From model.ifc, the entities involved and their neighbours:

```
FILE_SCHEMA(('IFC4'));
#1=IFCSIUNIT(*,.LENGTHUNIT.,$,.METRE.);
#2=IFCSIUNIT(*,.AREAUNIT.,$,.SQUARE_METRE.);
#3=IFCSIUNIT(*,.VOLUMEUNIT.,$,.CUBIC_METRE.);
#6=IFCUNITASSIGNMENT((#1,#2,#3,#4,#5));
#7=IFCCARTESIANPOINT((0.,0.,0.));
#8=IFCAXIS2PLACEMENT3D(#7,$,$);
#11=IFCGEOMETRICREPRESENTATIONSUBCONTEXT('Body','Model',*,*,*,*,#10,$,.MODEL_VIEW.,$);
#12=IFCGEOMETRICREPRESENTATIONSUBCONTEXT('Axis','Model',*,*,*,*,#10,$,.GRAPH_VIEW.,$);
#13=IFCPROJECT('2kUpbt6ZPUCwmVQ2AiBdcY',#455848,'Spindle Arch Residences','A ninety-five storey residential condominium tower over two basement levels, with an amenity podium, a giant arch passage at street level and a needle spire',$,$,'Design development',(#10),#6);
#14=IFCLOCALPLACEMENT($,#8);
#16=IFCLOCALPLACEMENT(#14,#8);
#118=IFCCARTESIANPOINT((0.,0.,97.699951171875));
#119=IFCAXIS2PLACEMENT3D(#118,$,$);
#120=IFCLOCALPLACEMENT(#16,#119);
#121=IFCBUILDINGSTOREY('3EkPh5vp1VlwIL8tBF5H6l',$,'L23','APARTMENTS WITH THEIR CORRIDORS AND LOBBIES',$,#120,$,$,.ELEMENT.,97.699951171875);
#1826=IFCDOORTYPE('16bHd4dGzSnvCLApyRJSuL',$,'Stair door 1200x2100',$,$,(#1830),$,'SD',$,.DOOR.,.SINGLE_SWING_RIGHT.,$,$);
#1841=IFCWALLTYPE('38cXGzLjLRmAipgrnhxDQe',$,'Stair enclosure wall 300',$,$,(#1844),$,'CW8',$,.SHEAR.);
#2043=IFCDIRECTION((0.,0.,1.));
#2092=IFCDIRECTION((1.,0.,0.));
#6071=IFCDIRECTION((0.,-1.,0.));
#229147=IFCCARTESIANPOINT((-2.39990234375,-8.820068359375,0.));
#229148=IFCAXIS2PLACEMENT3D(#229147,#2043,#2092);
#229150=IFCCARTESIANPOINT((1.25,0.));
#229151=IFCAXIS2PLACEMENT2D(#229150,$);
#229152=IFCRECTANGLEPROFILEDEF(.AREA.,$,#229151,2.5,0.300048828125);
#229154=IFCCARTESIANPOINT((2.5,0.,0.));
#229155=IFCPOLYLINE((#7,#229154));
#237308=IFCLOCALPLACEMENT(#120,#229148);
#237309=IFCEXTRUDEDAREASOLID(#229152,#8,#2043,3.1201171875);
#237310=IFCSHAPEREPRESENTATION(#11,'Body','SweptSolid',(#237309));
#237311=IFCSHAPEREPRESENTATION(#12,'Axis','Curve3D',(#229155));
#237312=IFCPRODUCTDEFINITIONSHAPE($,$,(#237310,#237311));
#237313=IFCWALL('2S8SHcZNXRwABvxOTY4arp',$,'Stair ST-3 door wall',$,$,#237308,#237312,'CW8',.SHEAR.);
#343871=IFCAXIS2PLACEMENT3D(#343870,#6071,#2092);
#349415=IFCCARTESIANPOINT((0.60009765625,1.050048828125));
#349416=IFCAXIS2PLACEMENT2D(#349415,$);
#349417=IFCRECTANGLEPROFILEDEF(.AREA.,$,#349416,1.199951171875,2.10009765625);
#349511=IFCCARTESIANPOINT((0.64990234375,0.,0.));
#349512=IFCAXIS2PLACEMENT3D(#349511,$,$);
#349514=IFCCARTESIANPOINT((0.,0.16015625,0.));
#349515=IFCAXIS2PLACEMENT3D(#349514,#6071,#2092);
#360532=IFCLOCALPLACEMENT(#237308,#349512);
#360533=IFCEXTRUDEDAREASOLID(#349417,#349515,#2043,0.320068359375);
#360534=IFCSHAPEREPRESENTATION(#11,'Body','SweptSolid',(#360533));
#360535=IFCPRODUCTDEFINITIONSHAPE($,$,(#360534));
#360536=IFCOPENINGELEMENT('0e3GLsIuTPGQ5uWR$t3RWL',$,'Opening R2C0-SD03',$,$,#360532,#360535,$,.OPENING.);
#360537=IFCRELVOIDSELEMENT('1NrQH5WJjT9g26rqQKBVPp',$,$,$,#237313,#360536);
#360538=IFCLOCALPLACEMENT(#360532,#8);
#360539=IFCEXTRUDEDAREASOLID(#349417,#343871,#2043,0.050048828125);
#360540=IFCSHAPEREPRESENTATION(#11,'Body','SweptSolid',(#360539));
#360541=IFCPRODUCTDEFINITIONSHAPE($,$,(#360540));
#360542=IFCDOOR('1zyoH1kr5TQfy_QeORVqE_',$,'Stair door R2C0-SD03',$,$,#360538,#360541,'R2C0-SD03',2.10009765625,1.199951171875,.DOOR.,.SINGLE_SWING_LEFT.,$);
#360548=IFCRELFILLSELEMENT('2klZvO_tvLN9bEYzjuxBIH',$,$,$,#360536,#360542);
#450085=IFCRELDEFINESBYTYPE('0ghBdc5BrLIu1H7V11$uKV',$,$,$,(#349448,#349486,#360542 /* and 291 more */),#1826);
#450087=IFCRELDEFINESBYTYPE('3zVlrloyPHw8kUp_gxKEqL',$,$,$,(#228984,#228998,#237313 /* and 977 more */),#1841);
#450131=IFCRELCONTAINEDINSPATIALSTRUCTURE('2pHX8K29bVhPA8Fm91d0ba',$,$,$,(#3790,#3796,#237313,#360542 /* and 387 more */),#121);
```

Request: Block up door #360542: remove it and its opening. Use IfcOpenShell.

```python
import ifcopenshell
import ifcopenshell.api.feature
import ifcopenshell.api.root
import ifcopenshell.geom
import ifcopenshell.util.shape

model = ifcopenshell.open("model.ifc")
settings = ifcopenshell.geom.settings()


def volume(element):
    """Net volume in cubic metres, openings subtracted."""
    shape = ifcopenshell.geom.create_shape(settings, element)
    return ifcopenshell.util.shape.get_volume(shape.geometry)


door = model.by_guid("1zyoH1kr5TQfy_QeORVqE_")
opening = door.FillsVoids[0].RelatingOpeningElement
wall = opening.VoidsElements[0].RelatingBuildingElement
before = volume(wall)

ifcopenshell.api.root.remove_product(model, product=door)
ifcopenshell.api.feature.remove_feature(model, feature=opening)

after = volume(wall)

print(f"wall volume {before:.3f} -> {after:.3f} m3")

model.write("model_v2.ifc")
```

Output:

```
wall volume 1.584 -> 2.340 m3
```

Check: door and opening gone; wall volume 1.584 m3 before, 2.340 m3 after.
